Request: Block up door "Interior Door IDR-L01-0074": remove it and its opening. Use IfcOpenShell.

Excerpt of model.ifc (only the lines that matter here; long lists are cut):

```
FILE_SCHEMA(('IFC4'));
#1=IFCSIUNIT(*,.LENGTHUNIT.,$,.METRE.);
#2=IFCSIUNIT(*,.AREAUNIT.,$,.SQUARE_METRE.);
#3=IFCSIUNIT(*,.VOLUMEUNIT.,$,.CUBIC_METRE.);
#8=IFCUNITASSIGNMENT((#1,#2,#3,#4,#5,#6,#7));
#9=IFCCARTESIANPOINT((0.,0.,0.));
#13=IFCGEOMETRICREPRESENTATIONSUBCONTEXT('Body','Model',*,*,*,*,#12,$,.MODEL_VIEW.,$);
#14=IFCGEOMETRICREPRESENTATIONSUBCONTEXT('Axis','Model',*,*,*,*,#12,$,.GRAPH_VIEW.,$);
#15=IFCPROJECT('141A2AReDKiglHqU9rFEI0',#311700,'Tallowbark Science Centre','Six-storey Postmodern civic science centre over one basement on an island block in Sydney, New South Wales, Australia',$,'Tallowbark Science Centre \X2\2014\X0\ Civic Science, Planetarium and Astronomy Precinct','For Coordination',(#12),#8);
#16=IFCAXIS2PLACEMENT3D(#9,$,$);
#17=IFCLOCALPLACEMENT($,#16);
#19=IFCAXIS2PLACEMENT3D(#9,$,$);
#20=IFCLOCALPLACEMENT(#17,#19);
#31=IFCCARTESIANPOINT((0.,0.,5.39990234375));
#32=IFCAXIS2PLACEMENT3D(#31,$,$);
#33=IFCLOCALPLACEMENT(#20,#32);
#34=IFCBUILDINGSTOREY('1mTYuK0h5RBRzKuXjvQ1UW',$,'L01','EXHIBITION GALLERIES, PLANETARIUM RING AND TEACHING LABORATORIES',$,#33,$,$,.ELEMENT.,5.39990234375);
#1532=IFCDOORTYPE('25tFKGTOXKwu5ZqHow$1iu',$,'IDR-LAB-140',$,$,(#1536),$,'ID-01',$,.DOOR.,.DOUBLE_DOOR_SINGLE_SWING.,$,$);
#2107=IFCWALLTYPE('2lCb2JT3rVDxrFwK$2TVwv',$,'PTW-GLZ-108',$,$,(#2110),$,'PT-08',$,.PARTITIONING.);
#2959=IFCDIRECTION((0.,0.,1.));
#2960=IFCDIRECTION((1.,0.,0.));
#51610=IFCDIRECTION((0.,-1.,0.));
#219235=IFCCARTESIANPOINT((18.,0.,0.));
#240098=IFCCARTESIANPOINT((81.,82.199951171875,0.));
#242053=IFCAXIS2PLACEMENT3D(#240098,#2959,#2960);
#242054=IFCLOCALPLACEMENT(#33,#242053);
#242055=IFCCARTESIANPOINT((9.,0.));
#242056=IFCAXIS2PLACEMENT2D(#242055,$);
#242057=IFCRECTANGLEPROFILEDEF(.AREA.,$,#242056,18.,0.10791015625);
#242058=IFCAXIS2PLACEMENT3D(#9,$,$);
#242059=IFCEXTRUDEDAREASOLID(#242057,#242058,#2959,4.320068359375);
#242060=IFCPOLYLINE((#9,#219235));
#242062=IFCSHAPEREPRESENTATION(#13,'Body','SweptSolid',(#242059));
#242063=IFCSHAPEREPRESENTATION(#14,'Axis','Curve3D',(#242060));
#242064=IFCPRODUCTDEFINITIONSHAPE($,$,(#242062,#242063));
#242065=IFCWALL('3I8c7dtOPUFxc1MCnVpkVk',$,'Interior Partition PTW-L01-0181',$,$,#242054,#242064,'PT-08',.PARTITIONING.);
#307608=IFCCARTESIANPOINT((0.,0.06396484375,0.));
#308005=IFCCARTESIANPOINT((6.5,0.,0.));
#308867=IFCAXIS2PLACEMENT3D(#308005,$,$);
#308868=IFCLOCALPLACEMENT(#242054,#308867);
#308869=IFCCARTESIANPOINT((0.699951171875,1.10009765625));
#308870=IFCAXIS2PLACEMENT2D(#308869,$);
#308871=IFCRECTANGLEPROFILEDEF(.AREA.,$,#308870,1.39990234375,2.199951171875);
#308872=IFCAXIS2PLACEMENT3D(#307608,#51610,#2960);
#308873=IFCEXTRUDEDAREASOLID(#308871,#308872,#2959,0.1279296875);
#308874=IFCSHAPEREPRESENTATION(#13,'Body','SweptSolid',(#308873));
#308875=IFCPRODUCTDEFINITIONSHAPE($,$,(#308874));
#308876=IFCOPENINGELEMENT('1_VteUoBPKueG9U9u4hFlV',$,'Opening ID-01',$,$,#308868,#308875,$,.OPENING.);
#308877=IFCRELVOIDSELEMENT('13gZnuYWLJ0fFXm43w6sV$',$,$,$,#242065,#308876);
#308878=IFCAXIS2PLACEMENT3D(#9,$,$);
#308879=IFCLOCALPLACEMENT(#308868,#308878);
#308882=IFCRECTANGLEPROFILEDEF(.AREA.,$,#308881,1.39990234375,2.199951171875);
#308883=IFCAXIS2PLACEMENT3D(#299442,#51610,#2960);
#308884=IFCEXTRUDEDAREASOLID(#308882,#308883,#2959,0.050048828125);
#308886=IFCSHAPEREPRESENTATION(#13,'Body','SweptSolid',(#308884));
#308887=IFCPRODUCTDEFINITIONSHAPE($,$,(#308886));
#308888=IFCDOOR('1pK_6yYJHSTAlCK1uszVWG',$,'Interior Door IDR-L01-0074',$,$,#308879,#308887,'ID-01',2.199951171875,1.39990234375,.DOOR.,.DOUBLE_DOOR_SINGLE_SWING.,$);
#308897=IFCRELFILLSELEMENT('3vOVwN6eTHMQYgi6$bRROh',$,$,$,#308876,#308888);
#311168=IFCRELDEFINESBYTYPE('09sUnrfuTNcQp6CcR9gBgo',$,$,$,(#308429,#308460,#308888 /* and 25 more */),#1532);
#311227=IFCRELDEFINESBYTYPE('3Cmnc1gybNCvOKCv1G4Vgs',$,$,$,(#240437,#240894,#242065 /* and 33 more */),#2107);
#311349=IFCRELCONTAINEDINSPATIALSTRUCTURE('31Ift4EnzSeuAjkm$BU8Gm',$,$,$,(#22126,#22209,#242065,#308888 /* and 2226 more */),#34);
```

```python
import ifcopenshell
import ifcopenshell.api.feature
import ifcopenshell.api.root
import ifcopenshell.geom
import ifcopenshell.util.shape

model = ifcopenshell.open("model.ifc")
settings = ifcopenshell.geom.settings()


def volume(element):
    """Net volume in cubic metres, openings subtracted."""
    shape = ifcopenshell.geom.create_shape(settings, element)
    return ifcopenshell.util.shape.get_volume(shape.geometry)


door = model.by_guid("1pK_6yYJHSTAlCK1uszVWG")
opening = door.FillsVoids[0].RelatingOpeningElement
wall = opening.VoidsElements[0].RelatingBuildingElement
before = volume(wall)

ifcopenshell.api.root.remove_product(model, product=door)
ifcopenshell.api.feature.remove_feature(model, feature=opening)

after = volume(wall)

print(f"wall volume {before:.3f} -> {after:.3f} m3")

model.write("model_rev.ifc")
```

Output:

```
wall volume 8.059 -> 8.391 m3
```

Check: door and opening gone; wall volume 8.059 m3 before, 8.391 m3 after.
